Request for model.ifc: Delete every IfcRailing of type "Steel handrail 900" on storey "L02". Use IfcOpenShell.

First a look at what the model holds.

```python
import ifcopenshell
import ifcopenshell.util.element

model = ifcopenshell.open("model.ifc")
print(model.schema)
storey = next(s for s in model.by_type("IfcBuildingStorey") if s.Name == "L02")
railings = [e for e in ifcopenshell.util.element.get_decomposition(storey) if e.is_a("IfcRailing")]
seen = {}
for e in railings:
    element_type = ifcopenshell.util.element.get_type(e)
    name = element_type.Name if element_type not in (None, e) else None
    seen[name] = seen.get(name, 0) + 1
for name, count in sorted(seen.items(), key=str):
    print(count, "x", name)
```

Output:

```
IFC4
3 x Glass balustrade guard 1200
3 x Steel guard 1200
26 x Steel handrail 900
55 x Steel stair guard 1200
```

```python
import ifcopenshell
import ifcopenshell.api.root
import ifcopenshell.util.element

model = ifcopenshell.open("model.ifc")

storey = next(s for s in model.by_type("IfcBuildingStorey") if s.Name == "L02")
railings = [e for e in ifcopenshell.util.element.get_decomposition(storey) if e.is_a("IfcRailing")]
targets = [e for e in railings if (t := ifcopenshell.util.element.get_type(e)) not in (None, e) and t.Name == "Steel handrail 900"]

for e in targets:
    ifcopenshell.api.root.remove_product(model, product=e)
print(len(targets), "removed")

model.write("model-out.ifc")
```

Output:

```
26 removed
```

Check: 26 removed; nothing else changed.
